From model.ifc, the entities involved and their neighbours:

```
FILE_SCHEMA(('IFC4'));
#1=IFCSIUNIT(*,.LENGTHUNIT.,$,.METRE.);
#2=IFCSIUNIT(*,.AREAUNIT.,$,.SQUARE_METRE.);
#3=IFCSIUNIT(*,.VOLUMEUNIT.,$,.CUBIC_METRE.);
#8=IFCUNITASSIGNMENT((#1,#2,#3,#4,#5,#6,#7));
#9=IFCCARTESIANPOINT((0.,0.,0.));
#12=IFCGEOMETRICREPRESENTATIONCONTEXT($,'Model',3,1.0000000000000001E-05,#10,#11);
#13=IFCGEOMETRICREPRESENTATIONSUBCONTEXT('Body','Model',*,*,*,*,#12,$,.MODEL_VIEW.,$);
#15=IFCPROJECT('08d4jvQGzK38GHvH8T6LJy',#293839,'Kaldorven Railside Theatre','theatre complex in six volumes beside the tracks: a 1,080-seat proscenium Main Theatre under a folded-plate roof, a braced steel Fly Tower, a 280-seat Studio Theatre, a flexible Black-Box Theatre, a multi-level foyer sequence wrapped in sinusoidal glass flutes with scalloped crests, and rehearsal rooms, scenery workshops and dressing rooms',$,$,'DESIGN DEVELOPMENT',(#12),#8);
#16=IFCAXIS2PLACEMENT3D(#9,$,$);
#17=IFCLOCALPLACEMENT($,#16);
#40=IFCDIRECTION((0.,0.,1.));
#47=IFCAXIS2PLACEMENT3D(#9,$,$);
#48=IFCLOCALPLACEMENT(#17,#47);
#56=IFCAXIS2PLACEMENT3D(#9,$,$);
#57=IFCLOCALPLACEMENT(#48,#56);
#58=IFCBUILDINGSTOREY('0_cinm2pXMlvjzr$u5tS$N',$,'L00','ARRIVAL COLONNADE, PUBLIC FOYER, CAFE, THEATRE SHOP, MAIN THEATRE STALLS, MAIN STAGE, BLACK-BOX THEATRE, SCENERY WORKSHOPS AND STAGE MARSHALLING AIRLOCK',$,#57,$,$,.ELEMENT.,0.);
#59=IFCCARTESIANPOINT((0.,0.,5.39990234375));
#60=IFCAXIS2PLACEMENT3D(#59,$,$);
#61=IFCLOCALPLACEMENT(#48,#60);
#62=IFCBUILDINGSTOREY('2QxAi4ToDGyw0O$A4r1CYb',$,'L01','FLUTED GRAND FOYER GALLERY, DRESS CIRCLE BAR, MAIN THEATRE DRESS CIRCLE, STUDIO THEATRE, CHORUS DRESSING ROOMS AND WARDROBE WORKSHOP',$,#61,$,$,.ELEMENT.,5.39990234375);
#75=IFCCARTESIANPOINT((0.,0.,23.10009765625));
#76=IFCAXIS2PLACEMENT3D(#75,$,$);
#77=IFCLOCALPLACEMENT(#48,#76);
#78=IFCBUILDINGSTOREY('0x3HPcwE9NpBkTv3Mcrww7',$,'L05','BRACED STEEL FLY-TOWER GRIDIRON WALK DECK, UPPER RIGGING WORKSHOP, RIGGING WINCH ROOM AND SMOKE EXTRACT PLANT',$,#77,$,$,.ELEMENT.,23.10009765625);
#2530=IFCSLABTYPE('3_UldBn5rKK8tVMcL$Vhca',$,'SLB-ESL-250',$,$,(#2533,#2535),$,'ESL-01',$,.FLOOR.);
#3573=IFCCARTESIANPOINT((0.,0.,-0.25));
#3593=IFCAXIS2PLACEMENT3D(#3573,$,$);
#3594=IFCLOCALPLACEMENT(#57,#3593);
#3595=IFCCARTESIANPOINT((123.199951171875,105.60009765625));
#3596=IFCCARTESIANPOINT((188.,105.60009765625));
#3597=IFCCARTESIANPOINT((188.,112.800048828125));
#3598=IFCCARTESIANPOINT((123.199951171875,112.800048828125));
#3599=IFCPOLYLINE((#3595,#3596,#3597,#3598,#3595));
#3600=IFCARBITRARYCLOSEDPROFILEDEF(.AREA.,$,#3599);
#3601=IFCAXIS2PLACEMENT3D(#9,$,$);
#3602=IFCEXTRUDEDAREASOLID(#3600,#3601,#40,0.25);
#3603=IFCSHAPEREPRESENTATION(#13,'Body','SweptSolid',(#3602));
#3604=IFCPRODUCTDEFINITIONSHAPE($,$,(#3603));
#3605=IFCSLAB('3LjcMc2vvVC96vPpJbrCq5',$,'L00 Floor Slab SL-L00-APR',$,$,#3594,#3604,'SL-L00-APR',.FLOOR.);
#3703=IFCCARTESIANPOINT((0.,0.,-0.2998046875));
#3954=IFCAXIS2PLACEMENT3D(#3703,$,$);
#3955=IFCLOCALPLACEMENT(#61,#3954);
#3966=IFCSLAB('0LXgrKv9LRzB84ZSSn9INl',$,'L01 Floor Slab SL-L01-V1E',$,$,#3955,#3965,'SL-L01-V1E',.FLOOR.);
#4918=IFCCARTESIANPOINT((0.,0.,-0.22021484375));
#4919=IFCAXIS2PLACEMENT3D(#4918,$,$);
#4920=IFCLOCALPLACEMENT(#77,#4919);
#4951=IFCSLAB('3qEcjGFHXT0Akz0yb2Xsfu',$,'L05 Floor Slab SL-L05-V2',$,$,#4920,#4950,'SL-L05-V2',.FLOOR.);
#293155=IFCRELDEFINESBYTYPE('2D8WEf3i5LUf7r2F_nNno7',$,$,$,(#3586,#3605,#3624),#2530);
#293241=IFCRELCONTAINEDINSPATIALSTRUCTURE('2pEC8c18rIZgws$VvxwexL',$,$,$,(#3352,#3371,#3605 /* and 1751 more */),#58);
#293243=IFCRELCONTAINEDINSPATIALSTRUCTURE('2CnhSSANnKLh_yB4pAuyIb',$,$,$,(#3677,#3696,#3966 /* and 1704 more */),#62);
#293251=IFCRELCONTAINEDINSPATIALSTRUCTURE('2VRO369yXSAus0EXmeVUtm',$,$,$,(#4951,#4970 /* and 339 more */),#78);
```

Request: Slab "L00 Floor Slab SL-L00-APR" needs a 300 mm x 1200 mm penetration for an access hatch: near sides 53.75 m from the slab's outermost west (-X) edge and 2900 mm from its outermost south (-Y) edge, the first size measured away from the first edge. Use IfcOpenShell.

```python
import numpy as np
import ifcopenshell
import ifcopenshell.api.feature
import ifcopenshell.api.geometry
import ifcopenshell.api.root
import ifcopenshell.geom
import ifcopenshell.util.placement
import ifcopenshell.util.representation
import ifcopenshell.util.shape
import ifcopenshell.util.unit

model = ifcopenshell.open("model.ifc")
unit_scale = ifcopenshell.util.unit.calculate_unit_scale(model)
settings = ifcopenshell.geom.settings()


def volume(element):
    """Net volume in cubic metres, openings subtracted."""
    shape = ifcopenshell.geom.create_shape(settings, element)
    return ifcopenshell.util.shape.get_volume(shape.geometry)


slab = model.by_guid("3LjcMc2vvVC96vPpJbrCq5")
before = volume(slab)

# Extent in the slab's own axes, in metres. The edges named are its -X and -Y sides.
slab_shape = ifcopenshell.geom.create_shape(settings, slab)
vertices = ifcopenshell.util.shape.get_vertices(slab_shape.geometry)
x_min, y_min, bottom = vertices.min(axis=0)
top = vertices[:, 2].max()

opening = ifcopenshell.api.root.create_entity(model, ifc_class="IfcOpeningElement", name="Access hatch opening", predefined_type="OPENING")
context = ifcopenshell.util.representation.get_context(model, "Model", "Body", "MODEL_VIEW")
width, depth = 0.3, 1.2
outline = [(0.0, 0.0), (width, 0.0), (width, depth), (0.0, depth), (0.0, 0.0)]
# Overshoot both faces by 50 mm so the cut is clean.
shape = ifcopenshell.api.geometry.add_slab_representation(
    model, context=context, depth=top - bottom + 0.1, polyline=outline
)
ifcopenshell.api.geometry.assign_representation(model, product=opening, representation=shape)

matrix = ifcopenshell.util.placement.get_local_placement(slab.ObjectPlacement)
matrix[:, 3] = matrix @ np.append(np.array([x_min + 53.75, y_min + 2.9, bottom - 0.05]) / unit_scale, 1.0)
ifcopenshell.api.geometry.edit_object_placement(model, product=opening, matrix=matrix, is_si=False)
ifcopenshell.api.feature.add_feature(model, feature=opening, element=slab)

after = volume(slab)

print(f"slab volume {before:.3f} -> {after:.3f} m3")

model.write("model_rev.ifc")
```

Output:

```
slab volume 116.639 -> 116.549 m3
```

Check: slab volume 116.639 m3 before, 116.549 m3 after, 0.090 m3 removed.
